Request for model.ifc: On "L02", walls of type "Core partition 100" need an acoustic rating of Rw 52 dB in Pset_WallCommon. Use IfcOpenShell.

First a look at what the model holds.

```python
import ifcopenshell
import ifcopenshell.util.element

model = ifcopenshell.open("model.ifc")
print(model.schema)
storey = next(s for s in model.by_type("IfcBuildingStorey") if s.Name == "L02")
walls = [e for e in ifcopenshell.util.element.get_decomposition(storey) if e.is_a("IfcWall")]
seen = {}
for e in walls:
    element_type = ifcopenshell.util.element.get_type(e)
    key = (element_type.Name if element_type != e and element_type else None, ifcopenshell.util.element.get_pset(e, "Pset_WallCommon", "AcousticRating"))
    seen[key] = seen.get(key, 0) + 1
for (name, value), count in sorted(seen.items(), key=str):
    print(count, "x", name, "|", value)
```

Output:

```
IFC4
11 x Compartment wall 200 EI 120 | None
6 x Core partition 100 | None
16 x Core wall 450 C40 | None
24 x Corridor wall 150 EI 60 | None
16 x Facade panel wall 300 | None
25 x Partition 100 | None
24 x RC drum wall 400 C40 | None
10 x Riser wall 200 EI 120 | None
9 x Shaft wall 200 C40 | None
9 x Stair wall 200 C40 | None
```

```python
import ifcopenshell
import ifcopenshell.api.pset
import ifcopenshell.util.element

model = ifcopenshell.open("model.ifc")

storey = next(s for s in model.by_type("IfcBuildingStorey") if s.Name == "L02")
walls = [e for e in ifcopenshell.util.element.get_decomposition(storey) if e.is_a("IfcWall")]

count = 0
for e in walls:
    element_type = ifcopenshell.util.element.get_type(e)
    if element_type in (None, e) or element_type.Name != "Core partition 100":
        continue
    # add_pset returns the element's existing set when there is one.
    pset = ifcopenshell.api.pset.add_pset(model, product=e, name="Pset_WallCommon")
    ifcopenshell.api.pset.edit_pset(model, pset=pset, properties={"AcousticRating": "Rw 52 dB"})
    count += 1

print(count, "walls updated")

model.write("model_updated.ifc")
```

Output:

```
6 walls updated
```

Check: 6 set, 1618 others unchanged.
